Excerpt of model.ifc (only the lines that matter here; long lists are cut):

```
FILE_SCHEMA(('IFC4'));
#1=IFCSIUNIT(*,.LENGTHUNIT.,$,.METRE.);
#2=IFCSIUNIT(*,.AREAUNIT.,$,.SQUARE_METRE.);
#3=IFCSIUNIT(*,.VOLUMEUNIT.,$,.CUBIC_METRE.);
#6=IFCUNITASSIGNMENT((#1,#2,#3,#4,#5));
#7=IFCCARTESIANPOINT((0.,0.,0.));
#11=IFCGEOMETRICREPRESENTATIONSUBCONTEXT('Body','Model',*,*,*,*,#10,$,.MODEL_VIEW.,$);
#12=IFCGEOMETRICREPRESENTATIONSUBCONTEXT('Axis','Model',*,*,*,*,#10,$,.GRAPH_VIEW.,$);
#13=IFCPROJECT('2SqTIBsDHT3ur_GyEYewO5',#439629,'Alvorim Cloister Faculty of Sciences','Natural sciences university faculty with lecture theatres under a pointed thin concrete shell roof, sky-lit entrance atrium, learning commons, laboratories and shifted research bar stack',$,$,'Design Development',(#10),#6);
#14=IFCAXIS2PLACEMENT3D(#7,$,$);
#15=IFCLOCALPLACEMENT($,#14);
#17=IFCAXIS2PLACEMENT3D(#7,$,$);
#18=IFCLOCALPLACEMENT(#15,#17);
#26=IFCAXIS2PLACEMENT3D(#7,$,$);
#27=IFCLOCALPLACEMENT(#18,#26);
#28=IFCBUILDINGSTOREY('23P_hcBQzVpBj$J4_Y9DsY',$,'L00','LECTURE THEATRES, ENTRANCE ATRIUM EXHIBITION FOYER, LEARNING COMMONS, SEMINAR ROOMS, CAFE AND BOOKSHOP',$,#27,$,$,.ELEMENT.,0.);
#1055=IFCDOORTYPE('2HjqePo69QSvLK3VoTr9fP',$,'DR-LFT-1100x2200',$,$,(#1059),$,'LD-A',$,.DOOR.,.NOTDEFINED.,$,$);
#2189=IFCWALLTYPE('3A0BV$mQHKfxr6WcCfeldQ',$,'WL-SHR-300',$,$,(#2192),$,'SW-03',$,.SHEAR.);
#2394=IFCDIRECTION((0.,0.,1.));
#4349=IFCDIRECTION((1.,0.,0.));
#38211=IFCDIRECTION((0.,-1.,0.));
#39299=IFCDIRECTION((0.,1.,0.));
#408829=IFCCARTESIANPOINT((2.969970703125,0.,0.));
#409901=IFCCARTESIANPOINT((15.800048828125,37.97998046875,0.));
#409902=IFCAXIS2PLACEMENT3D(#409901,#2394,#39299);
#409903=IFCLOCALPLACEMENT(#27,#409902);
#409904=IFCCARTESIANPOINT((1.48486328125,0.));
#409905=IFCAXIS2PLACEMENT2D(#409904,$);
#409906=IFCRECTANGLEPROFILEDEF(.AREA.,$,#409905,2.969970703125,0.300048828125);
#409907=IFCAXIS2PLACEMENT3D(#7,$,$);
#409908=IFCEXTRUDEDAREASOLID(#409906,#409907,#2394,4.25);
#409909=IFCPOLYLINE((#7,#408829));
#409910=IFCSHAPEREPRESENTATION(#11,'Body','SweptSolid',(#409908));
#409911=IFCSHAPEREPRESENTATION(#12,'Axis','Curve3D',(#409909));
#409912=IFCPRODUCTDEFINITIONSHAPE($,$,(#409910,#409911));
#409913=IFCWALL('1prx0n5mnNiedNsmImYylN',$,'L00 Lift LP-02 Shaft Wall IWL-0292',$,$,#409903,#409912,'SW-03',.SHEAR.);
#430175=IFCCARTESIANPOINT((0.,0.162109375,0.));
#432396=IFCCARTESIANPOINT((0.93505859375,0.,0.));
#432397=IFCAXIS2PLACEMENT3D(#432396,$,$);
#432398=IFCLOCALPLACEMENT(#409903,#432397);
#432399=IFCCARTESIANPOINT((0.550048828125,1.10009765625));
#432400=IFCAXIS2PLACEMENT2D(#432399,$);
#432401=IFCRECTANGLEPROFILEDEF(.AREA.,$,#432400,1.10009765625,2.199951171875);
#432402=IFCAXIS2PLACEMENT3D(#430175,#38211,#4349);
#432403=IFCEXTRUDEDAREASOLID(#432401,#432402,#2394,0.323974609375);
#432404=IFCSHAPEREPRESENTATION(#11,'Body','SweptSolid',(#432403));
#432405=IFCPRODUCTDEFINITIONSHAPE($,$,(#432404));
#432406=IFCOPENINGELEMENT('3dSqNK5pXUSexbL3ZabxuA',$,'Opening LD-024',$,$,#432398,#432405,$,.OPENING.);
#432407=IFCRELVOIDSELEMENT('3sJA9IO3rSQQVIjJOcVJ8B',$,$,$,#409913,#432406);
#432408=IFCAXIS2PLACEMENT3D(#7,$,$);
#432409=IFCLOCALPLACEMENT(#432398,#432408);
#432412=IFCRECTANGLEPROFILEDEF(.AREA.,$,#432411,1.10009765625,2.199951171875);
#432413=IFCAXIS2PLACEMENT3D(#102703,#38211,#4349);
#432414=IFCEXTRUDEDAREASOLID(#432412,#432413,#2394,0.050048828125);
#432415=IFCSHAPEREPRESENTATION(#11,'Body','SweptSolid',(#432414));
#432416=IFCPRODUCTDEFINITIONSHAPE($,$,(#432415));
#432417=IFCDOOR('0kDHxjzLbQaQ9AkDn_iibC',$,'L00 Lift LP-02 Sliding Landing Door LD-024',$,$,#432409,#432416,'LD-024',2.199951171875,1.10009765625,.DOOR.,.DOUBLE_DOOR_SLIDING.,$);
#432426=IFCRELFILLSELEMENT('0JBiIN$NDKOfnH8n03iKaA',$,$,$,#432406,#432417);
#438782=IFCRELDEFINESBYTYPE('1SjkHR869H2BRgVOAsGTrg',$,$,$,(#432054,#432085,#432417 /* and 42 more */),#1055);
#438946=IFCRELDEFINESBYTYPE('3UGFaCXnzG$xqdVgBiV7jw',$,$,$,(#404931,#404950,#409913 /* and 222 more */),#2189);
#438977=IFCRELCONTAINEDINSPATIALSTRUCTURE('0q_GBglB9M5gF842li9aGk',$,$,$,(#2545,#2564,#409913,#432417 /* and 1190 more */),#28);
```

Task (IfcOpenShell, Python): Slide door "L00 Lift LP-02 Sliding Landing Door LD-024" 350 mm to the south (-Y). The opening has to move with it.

```python
import ifcopenshell
import ifcopenshell.api.geometry
import ifcopenshell.util.placement

model = ifcopenshell.open("model.ifc")

door = model.by_guid("0kDHxjzLbQaQ9AkDn_iibC")
opening = door.FillsVoids[0].RelatingOpeningElement
wall = opening.VoidsElements[0].RelatingBuildingElement

wall_matrix = ifcopenshell.util.placement.get_local_placement(wall.ObjectPlacement)
shift = wall_matrix[:3, 0] * -0.35
before = ifcopenshell.util.placement.get_local_placement(door.ObjectPlacement)[:3, 3].copy()

# The door is placed relative to its opening, so it follows when the opening moves.
matrix = ifcopenshell.util.placement.get_local_placement(opening.ObjectPlacement)
matrix[:3, 3] += shift
ifcopenshell.api.geometry.edit_object_placement(
    model, product=opening, matrix=matrix, is_si=False, should_transform_children=True
)

after = ifcopenshell.util.placement.get_local_placement(door.ObjectPlacement)[:3, 3]
print("door moved by", (after - before).round(3) + 0.0)

model.write("model_v2.ifc")
```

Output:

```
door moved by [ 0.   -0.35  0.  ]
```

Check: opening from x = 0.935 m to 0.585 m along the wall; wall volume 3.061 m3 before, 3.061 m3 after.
